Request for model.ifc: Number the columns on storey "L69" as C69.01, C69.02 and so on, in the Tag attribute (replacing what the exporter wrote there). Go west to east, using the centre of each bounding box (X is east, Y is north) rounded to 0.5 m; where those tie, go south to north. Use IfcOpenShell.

First a look at what the model holds.

```python
import ifcopenshell
import ifcopenshell.util.element
import ifcopenshell.util.placement

model = ifcopenshell.open("model.ifc")
print(model.schema)
storey = next(s for s in model.by_type("IfcBuildingStorey") if s.Name == "L69")
columns = [e for e in ifcopenshell.util.element.get_decomposition(storey) if e.is_a("IfcColumn")]
for e in sorted(columns, key=lambda e: e.id()):
    origin = ifcopenshell.util.placement.get_local_placement(e.ObjectPlacement)[:3, 3]
    print(e.id(), e.Tag, e.Name, origin.round(2) + 0.0, sep=" | ")
```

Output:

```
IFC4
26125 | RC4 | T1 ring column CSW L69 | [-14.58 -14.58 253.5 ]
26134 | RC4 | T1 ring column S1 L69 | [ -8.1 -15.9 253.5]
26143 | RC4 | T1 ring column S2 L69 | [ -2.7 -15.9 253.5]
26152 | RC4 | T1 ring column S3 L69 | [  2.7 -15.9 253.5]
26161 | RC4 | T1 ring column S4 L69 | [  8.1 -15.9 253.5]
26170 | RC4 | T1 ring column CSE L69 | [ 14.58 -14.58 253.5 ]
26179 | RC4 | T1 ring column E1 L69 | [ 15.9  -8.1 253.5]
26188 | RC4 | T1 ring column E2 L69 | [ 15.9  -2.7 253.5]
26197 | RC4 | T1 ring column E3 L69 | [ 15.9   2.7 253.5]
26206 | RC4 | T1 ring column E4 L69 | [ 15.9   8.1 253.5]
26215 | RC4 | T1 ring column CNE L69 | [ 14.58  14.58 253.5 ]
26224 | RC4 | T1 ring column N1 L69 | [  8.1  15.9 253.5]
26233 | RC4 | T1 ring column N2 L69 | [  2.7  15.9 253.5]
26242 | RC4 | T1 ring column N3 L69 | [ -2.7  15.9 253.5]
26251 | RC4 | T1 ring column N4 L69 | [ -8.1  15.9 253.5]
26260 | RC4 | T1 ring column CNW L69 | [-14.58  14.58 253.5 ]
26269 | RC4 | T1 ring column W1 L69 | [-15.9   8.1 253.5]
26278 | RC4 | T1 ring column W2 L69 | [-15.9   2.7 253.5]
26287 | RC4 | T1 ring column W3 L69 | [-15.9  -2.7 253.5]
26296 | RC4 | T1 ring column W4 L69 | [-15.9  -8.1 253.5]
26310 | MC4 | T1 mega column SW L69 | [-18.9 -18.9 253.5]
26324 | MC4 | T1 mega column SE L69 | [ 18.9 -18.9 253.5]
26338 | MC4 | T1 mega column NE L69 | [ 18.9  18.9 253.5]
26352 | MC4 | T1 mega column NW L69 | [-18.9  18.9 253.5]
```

```python
import ifcopenshell
import ifcopenshell.geom
import ifcopenshell.util.element
import ifcopenshell.util.shape

model = ifcopenshell.open("model.ifc")
settings = ifcopenshell.geom.settings()
settings.set("use-world-coords", True)


def centre(element):
    shape = ifcopenshell.geom.create_shape(settings, element)
    return ifcopenshell.util.shape.get_bbox_centroid(shape.geometry)


storey = next(s for s in model.by_type("IfcBuildingStorey") if s.Name == "L69")
columns = [e for e in ifcopenshell.util.element.get_decomposition(storey) if e.is_a("IfcColumn")]

# Insertion points can sit at a corner or the storey origin, so sort by the geometry (in metres).
centres = {e: centre(e) for e in columns}
columns.sort(key=lambda e: (round(centres[e][0] / 0.5), centres[e][1]))

for i, e in enumerate(columns, start=1):
    number = f"C69.{i:02d}"
    e.Tag = number
    print(e.id(), number)

model.write("model_edited.ifc")
```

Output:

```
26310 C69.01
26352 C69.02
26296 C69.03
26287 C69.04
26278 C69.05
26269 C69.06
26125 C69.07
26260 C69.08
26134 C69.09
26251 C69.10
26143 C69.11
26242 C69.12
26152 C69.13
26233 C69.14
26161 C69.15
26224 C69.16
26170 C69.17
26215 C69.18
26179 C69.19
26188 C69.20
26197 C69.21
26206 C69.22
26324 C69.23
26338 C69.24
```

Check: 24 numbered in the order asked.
